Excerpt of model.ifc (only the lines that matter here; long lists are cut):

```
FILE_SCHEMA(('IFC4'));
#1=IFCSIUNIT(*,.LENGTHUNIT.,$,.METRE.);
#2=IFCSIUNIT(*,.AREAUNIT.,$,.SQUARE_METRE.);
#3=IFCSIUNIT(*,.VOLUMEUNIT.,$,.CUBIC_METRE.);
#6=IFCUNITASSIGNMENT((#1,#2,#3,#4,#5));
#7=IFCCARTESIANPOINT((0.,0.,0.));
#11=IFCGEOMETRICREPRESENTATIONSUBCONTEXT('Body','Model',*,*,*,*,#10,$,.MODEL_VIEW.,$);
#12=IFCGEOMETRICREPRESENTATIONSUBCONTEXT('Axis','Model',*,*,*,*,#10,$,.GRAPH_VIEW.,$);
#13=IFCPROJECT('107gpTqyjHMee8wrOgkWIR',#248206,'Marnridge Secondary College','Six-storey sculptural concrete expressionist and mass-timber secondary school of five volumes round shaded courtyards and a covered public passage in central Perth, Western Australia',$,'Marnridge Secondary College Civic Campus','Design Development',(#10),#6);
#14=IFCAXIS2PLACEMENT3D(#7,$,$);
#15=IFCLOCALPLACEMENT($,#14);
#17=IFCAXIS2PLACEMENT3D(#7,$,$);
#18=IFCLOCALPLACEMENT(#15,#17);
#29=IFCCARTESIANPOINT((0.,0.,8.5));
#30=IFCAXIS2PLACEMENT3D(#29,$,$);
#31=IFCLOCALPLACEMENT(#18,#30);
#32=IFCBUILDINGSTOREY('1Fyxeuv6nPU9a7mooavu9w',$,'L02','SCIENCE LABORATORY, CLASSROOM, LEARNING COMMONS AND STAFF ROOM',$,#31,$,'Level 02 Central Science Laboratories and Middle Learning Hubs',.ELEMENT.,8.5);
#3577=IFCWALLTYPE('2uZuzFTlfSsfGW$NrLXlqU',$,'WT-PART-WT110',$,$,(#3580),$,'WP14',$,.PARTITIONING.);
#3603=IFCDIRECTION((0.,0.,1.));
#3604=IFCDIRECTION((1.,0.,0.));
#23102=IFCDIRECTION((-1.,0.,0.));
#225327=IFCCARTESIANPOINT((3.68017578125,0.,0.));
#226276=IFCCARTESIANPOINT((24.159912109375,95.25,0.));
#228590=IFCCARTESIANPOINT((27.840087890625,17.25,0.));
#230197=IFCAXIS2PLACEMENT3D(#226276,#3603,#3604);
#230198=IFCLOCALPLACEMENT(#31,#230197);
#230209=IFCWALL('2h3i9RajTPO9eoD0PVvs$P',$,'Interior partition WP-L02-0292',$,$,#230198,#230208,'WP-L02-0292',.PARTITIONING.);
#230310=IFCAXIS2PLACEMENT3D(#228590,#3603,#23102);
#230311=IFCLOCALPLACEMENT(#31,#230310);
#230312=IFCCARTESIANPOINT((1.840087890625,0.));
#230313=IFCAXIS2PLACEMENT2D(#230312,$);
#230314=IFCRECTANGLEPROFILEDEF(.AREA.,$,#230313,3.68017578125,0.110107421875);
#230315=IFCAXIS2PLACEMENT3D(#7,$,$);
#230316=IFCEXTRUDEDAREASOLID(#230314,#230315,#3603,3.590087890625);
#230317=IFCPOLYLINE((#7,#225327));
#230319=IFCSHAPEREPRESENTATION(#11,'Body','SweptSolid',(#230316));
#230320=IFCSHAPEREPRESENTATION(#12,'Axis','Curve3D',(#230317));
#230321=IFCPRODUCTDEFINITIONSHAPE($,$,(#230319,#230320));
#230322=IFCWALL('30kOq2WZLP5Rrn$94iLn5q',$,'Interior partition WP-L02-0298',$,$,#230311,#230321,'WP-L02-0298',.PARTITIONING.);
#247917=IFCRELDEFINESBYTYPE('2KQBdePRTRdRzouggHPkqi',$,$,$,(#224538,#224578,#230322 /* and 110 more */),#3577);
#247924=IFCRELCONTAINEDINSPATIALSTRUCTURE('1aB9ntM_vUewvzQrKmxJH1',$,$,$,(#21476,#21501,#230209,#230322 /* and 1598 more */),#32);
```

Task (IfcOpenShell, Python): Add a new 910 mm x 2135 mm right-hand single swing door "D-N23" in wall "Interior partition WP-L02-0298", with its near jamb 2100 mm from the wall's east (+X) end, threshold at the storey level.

```python
import numpy as np
import ifcopenshell
import ifcopenshell.api.feature
import ifcopenshell.api.geometry
import ifcopenshell.api.root
import ifcopenshell.api.spatial
import ifcopenshell.geom
import ifcopenshell.util.element
import ifcopenshell.util.placement
import ifcopenshell.util.representation
import ifcopenshell.util.shape
import ifcopenshell.util.unit

model = ifcopenshell.open("model.ifc")
unit_scale = ifcopenshell.util.unit.calculate_unit_scale(model)
settings = ifcopenshell.geom.settings()


def volume(element):
    """Net volume in cubic metres, openings subtracted."""
    shape = ifcopenshell.geom.create_shape(settings, element)
    return ifcopenshell.util.shape.get_volume(shape.geometry)


wall = model.by_guid("30kOq2WZLP5Rrn$94iLn5q")
storey = ifcopenshell.util.element.get_container(wall, ifc_class="IfcBuildingStorey")
context = ifcopenshell.util.representation.get_context(model, "Model", "Body", "MODEL_VIEW")
before = volume(wall)

width, height, from_end, sill = 0.91, 2.135, 2.1, 0.0  # metres

# The wall runs along its own X axis, and the end named is its -X end.
wall_shape = ifcopenshell.geom.create_shape(settings, wall)
x, y, z = ifcopenshell.util.shape.get_vertices(wall_shape.geometry).T
start = x.min() + from_end
face, thickness = float(y.min()), float(y.max() - y.min())
wall_matrix = ifcopenshell.util.placement.get_local_placement(wall.ObjectPlacement)
level = ifcopenshell.util.placement.get_local_placement(storey.ObjectPlacement)[2, 3]


def in_wall(x, y):
    """Placement at x, y metres in the wall's axes, at sill height."""
    matrix = wall_matrix.copy()
    matrix[:, 3] = wall_matrix @ np.array([x / unit_scale, y / unit_scale, 0.0, 1.0])
    matrix[2, 3] = level + sill / unit_scale
    return matrix


# Opening: a box that overshoots both wall faces by 50 mm.
opening = ifcopenshell.api.root.create_entity(model, ifc_class="IfcOpeningElement", predefined_type="OPENING")
box = ifcopenshell.api.geometry.add_wall_representation(
    model, context=context, length=width, height=height, thickness=thickness + 0.1
)
ifcopenshell.api.geometry.assign_representation(model, product=opening, representation=box)
ifcopenshell.api.geometry.edit_object_placement(model, product=opening, matrix=in_wall(start, face - 0.05), is_si=False)
ifcopenshell.api.feature.add_feature(model, feature=opening, element=wall)

door = ifcopenshell.api.root.create_entity(model, ifc_class="IfcDoor", name="D-N23", predefined_type="DOOR")
door.OverallWidth, door.OverallHeight = width / unit_scale, height / unit_scale
door.OperationType = "SINGLE_SWING_RIGHT"
body = ifcopenshell.api.geometry.add_door_representation(
    model,
    context=context,
    overall_width=door.OverallWidth,
    overall_height=door.OverallHeight,
    operation_type="SINGLE_SWING_RIGHT",
    lining_properties={"LiningDepth": thickness / unit_scale, "ThresholdDepth": thickness / unit_scale},
)
ifcopenshell.api.geometry.assign_representation(model, product=door, representation=body)
ifcopenshell.api.spatial.assign_container(model, products=[door], relating_structure=storey)
ifcopenshell.api.feature.add_filling(model, opening=opening, element=door)

# The lining spans the wall, so the door starts at the wall face.
ifcopenshell.api.geometry.edit_object_placement(model, product=door, matrix=in_wall(start, face), is_si=False)

after = volume(wall)

print(f"wall volume {before:.3f} -> {after:.3f} m3")

model.write("model_rev.ifc")
```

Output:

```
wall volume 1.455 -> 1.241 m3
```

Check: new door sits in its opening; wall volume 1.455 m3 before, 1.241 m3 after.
